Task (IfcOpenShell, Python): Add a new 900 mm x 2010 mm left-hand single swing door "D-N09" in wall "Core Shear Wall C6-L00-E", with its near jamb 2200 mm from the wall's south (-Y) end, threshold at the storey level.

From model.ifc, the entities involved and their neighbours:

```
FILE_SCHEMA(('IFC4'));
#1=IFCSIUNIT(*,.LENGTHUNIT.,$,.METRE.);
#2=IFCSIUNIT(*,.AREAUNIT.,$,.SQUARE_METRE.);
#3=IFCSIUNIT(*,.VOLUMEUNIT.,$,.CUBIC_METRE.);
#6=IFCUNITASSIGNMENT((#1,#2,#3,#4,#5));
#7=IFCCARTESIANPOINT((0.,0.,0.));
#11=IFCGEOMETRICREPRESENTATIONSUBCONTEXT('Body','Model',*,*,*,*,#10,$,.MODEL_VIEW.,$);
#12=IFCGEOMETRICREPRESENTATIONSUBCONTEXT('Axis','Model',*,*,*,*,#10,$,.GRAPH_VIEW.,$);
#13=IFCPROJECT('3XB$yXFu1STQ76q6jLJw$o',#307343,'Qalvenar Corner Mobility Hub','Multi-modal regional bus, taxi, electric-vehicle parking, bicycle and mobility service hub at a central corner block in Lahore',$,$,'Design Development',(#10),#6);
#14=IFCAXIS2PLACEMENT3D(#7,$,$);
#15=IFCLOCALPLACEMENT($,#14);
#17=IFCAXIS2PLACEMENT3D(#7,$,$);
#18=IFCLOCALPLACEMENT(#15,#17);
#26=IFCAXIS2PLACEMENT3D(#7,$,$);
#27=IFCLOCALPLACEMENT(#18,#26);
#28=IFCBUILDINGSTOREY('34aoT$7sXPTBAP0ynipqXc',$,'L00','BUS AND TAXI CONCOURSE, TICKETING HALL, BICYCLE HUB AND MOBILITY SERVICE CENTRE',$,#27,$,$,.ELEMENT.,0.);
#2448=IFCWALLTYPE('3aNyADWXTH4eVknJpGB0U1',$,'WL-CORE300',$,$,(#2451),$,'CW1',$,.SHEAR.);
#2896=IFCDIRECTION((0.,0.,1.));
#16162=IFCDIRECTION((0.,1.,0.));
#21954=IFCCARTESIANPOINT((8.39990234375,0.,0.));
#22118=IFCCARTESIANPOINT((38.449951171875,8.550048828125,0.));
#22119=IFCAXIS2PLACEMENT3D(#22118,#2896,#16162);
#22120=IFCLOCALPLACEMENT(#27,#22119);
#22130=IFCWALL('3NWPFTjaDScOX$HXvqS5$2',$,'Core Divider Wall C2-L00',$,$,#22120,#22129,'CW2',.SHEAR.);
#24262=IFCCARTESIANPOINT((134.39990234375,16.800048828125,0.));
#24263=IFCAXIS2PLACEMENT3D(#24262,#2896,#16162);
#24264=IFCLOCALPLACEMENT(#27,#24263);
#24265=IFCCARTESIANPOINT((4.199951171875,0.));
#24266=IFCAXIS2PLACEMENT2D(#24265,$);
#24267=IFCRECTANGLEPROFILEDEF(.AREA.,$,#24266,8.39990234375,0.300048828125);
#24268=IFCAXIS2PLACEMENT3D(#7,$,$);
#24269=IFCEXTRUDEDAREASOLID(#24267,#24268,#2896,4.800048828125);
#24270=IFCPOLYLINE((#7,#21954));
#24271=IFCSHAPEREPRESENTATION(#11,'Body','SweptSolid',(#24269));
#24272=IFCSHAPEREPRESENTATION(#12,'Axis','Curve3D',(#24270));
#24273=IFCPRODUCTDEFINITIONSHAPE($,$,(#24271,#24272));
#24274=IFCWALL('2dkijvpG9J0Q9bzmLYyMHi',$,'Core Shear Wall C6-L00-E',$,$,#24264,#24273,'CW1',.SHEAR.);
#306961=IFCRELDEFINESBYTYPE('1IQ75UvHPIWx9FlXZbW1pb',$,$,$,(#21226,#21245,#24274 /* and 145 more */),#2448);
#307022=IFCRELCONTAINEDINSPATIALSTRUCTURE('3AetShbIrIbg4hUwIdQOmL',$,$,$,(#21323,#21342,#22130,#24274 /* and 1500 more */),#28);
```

```python
import numpy as np
import ifcopenshell
import ifcopenshell.api.feature
import ifcopenshell.api.geometry
import ifcopenshell.api.root
import ifcopenshell.api.spatial
import ifcopenshell.geom
import ifcopenshell.util.element
import ifcopenshell.util.placement
import ifcopenshell.util.representation
import ifcopenshell.util.shape
import ifcopenshell.util.unit

model = ifcopenshell.open("model.ifc")
unit_scale = ifcopenshell.util.unit.calculate_unit_scale(model)
settings = ifcopenshell.geom.settings()


def volume(element):
    """Net volume in cubic metres, openings subtracted."""
    shape = ifcopenshell.geom.create_shape(settings, element)
    return ifcopenshell.util.shape.get_volume(shape.geometry)


wall = model.by_id(24274)
storey = ifcopenshell.util.element.get_container(wall, ifc_class="IfcBuildingStorey")
context = ifcopenshell.util.representation.get_context(model, "Model", "Body", "MODEL_VIEW")
before = volume(wall)

width, height, from_end, sill = 0.9, 2.01, 2.2, 0.0  # metres

# The wall runs along its own X axis, and the end named is its -X end.
wall_shape = ifcopenshell.geom.create_shape(settings, wall)
x, y, z = ifcopenshell.util.shape.get_vertices(wall_shape.geometry).T
start = x.min() + from_end
face, thickness = float(y.min()), float(y.max() - y.min())
wall_matrix = ifcopenshell.util.placement.get_local_placement(wall.ObjectPlacement)
level = ifcopenshell.util.placement.get_local_placement(storey.ObjectPlacement)[2, 3]


def in_wall(x, y):
    """Placement at x, y metres in the wall's axes, at sill height."""
    matrix = wall_matrix.copy()
    matrix[:, 3] = wall_matrix @ np.array([x / unit_scale, y / unit_scale, 0.0, 1.0])
    matrix[2, 3] = level + sill / unit_scale
    return matrix


# Opening: a box that overshoots both wall faces by 50 mm.
opening = ifcopenshell.api.root.create_entity(model, ifc_class="IfcOpeningElement", predefined_type="OPENING")
box = ifcopenshell.api.geometry.add_wall_representation(
    model, context=context, length=width, height=height, thickness=thickness + 0.1
)
ifcopenshell.api.geometry.assign_representation(model, product=opening, representation=box)
ifcopenshell.api.geometry.edit_object_placement(model, product=opening, matrix=in_wall(start, face - 0.05), is_si=False)
ifcopenshell.api.feature.add_feature(model, feature=opening, element=wall)

door = ifcopenshell.api.root.create_entity(model, ifc_class="IfcDoor", name="D-N09", predefined_type="DOOR")
door.OverallWidth, door.OverallHeight = width / unit_scale, height / unit_scale
door.OperationType = "SINGLE_SWING_LEFT"
body = ifcopenshell.api.geometry.add_door_representation(
    model,
    context=context,
    overall_width=door.OverallWidth,
    overall_height=door.OverallHeight,
    operation_type="SINGLE_SWING_LEFT",
    lining_properties={"LiningDepth": thickness / unit_scale, "ThresholdDepth": thickness / unit_scale},
)
ifcopenshell.api.geometry.assign_representation(model, product=door, representation=body)
ifcopenshell.api.spatial.assign_container(model, products=[door], relating_structure=storey)
ifcopenshell.api.feature.add_filling(model, opening=opening, element=door)

# The lining spans the wall, so the door starts at the wall face.
ifcopenshell.api.geometry.edit_object_placement(model, product=door, matrix=in_wall(start, face), is_si=False)

after = volume(wall)

print(f"wall volume {before:.3f} -> {after:.3f} m3")

model.write("model_v2.ifc")
```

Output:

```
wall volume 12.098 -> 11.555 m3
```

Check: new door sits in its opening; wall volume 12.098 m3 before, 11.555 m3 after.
